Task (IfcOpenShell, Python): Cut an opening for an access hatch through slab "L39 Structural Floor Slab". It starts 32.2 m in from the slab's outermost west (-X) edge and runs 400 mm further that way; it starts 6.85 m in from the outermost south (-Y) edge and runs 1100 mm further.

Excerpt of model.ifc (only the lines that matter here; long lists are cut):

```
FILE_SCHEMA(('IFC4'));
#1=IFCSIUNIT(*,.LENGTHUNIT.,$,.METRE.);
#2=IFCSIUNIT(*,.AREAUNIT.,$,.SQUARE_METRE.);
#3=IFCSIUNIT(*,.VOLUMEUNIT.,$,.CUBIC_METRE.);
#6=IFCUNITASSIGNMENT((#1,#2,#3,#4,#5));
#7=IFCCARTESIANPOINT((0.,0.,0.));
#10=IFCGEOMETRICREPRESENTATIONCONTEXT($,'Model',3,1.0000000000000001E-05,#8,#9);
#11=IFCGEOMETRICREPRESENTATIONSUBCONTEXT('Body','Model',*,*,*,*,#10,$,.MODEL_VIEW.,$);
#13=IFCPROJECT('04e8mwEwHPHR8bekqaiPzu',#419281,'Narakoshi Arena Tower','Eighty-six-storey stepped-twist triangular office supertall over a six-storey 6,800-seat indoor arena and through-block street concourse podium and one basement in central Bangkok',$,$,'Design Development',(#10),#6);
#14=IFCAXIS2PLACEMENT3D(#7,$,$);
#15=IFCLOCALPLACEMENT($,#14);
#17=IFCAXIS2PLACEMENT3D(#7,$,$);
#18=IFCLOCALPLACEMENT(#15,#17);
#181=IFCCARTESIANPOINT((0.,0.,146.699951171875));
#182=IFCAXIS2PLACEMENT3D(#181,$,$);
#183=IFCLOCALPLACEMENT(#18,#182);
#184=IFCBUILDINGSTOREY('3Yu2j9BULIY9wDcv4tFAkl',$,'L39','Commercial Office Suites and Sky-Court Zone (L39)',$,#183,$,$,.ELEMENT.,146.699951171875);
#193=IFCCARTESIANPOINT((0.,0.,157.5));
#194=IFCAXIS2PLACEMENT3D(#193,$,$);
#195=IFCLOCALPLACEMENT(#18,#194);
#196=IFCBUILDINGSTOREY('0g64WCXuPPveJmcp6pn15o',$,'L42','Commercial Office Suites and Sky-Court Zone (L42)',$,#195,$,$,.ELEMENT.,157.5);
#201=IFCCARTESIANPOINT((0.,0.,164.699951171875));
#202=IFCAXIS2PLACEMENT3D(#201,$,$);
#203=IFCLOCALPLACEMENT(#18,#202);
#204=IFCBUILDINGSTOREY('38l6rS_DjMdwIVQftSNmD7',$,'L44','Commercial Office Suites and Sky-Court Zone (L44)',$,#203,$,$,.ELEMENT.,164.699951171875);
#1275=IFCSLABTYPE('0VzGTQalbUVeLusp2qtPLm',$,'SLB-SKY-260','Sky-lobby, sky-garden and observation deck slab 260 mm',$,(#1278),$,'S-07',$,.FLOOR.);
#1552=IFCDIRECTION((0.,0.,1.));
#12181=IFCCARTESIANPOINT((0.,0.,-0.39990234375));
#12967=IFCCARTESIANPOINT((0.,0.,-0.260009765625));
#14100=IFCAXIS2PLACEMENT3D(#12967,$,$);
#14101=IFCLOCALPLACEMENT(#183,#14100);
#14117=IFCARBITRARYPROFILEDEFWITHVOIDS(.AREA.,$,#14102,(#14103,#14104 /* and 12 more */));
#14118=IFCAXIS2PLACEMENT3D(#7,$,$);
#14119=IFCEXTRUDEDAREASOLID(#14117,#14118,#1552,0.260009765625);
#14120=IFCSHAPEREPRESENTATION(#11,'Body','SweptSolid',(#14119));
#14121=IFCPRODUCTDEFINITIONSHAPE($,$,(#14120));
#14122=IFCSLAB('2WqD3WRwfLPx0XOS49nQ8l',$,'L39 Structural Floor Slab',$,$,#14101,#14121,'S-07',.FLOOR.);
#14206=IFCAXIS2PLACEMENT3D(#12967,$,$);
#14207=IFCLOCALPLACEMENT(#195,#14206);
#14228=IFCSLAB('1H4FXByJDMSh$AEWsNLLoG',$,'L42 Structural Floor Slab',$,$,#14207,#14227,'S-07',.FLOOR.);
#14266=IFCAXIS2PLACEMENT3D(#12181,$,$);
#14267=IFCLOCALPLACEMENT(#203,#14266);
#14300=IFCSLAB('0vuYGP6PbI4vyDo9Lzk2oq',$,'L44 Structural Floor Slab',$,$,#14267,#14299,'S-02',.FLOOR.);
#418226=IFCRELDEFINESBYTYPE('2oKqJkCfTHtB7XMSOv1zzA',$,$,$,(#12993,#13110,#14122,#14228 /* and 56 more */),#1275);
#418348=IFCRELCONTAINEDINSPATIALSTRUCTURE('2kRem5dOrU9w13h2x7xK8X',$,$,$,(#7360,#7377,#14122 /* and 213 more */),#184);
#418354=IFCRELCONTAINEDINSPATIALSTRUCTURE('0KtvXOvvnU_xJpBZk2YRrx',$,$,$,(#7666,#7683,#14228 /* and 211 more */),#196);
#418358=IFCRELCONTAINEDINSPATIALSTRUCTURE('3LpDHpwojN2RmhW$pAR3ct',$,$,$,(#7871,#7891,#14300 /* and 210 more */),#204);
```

```python
import numpy as np
import ifcopenshell
import ifcopenshell.api.feature
import ifcopenshell.api.geometry
import ifcopenshell.api.root
import ifcopenshell.geom
import ifcopenshell.util.placement
import ifcopenshell.util.representation
import ifcopenshell.util.shape
import ifcopenshell.util.unit

model = ifcopenshell.open("model.ifc")
unit_scale = ifcopenshell.util.unit.calculate_unit_scale(model)
settings = ifcopenshell.geom.settings()


def volume(element):
    """Net volume in cubic metres, openings subtracted."""
    shape = ifcopenshell.geom.create_shape(settings, element)
    return ifcopenshell.util.shape.get_volume(shape.geometry)


slab = model.by_id(14122)
before = volume(slab)

# Extent in the slab's own axes, in metres. The edges named are its -X and -Y sides.
slab_shape = ifcopenshell.geom.create_shape(settings, slab)
vertices = ifcopenshell.util.shape.get_vertices(slab_shape.geometry)
x_min, y_min, bottom = vertices.min(axis=0)
top = vertices[:, 2].max()

opening = ifcopenshell.api.root.create_entity(model, ifc_class="IfcOpeningElement", name="Access hatch opening", predefined_type="OPENING")
context = ifcopenshell.util.representation.get_context(model, "Model", "Body", "MODEL_VIEW")
width, depth = 0.4, 1.1
outline = [(0.0, 0.0), (width, 0.0), (width, depth), (0.0, depth), (0.0, 0.0)]
# Overshoot both faces by 50 mm so the cut is clean.
shape = ifcopenshell.api.geometry.add_slab_representation(
    model, context=context, depth=top - bottom + 0.1, polyline=outline
)
ifcopenshell.api.geometry.assign_representation(model, product=opening, representation=shape)

matrix = ifcopenshell.util.placement.get_local_placement(slab.ObjectPlacement)
matrix[:, 3] = matrix @ np.append(np.array([x_min + 32.2, y_min + 6.85, bottom - 0.05]) / unit_scale, 1.0)
ifcopenshell.api.geometry.edit_object_placement(model, product=opening, matrix=matrix, is_si=False)
ifcopenshell.api.feature.add_feature(model, feature=opening, element=slab)

after = volume(slab)

print(f"slab volume {before:.3f} -> {after:.3f} m3")

model.write("model_edited.ifc")
```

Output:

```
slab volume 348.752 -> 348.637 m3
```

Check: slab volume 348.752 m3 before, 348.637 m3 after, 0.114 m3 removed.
